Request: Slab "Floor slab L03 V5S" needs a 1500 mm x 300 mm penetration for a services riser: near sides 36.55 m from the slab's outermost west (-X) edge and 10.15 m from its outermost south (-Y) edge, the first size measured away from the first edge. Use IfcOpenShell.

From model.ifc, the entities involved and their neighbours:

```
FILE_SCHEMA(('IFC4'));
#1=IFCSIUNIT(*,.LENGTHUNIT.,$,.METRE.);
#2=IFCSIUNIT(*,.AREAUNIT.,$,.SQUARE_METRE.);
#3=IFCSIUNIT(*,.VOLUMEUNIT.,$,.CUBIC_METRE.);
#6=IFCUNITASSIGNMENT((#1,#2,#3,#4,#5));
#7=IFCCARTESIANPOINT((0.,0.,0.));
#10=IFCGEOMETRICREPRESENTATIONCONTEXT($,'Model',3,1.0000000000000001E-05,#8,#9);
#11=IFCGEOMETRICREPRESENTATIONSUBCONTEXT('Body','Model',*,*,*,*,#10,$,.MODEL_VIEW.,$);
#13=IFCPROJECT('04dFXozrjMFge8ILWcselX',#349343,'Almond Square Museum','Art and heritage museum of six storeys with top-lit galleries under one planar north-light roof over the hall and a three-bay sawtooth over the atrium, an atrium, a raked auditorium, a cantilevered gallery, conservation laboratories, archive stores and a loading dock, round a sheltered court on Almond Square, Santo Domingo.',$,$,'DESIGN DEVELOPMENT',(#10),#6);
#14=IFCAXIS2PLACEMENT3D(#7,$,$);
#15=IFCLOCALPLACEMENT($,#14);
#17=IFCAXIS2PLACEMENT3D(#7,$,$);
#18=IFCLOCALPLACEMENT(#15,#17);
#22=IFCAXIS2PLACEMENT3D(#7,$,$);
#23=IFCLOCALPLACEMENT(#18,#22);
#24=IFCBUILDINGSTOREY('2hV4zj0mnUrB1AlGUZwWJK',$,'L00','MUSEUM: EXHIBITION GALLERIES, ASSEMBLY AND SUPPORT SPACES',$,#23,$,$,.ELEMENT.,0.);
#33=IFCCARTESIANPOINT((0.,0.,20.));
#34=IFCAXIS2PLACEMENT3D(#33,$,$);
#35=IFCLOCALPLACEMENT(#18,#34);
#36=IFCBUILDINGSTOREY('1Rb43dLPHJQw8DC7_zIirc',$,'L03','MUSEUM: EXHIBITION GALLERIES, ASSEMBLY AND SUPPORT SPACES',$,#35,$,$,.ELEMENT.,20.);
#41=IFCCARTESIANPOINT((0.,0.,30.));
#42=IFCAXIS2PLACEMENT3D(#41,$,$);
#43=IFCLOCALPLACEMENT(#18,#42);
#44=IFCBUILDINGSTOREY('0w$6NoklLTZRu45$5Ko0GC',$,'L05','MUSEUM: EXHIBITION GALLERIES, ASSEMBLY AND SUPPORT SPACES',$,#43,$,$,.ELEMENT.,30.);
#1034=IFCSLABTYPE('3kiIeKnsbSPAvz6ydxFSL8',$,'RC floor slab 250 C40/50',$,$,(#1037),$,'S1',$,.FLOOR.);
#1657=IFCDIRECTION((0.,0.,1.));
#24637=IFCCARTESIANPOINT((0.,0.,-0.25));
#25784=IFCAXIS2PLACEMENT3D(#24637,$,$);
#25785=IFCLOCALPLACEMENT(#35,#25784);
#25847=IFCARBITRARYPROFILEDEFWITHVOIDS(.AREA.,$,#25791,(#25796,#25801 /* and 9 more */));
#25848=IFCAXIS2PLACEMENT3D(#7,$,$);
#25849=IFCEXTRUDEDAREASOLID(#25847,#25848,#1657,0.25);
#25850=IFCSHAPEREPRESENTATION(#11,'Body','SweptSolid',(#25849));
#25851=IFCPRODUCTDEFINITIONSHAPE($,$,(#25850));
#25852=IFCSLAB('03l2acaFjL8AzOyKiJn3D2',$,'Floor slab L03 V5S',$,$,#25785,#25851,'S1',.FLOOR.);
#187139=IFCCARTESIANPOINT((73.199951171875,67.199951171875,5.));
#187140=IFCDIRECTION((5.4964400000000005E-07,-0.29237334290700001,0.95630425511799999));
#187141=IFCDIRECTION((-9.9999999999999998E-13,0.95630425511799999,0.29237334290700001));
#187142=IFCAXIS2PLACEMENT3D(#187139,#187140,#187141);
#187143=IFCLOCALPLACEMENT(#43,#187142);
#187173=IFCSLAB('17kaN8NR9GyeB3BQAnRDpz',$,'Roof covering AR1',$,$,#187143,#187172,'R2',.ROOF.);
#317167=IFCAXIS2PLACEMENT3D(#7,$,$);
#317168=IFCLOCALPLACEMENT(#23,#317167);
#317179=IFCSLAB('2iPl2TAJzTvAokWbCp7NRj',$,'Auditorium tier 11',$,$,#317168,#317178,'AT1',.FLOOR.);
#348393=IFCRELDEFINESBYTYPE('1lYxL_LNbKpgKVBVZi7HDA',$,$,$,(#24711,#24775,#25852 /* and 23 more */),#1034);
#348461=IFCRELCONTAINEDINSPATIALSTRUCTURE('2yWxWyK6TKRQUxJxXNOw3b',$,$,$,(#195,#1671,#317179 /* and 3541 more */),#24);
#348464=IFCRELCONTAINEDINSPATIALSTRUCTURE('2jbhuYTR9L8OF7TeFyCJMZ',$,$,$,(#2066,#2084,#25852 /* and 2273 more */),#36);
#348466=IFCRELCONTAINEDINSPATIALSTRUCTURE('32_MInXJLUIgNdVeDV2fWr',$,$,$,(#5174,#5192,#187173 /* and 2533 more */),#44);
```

```python
import numpy as np
import ifcopenshell
import ifcopenshell.api.feature
import ifcopenshell.api.geometry
import ifcopenshell.api.root
import ifcopenshell.geom
import ifcopenshell.util.placement
import ifcopenshell.util.representation
import ifcopenshell.util.shape
import ifcopenshell.util.unit

model = ifcopenshell.open("model.ifc")
unit_scale = ifcopenshell.util.unit.calculate_unit_scale(model)
settings = ifcopenshell.geom.settings()


def volume(element):
    """Net volume in cubic metres, openings subtracted."""
    shape = ifcopenshell.geom.create_shape(settings, element)
    return ifcopenshell.util.shape.get_volume(shape.geometry)


slab = model.by_id(25852)
before = volume(slab)

# Extent in the slab's own axes, in metres. The edges named are its -X and -Y sides.
slab_shape = ifcopenshell.geom.create_shape(settings, slab)
vertices = ifcopenshell.util.shape.get_vertices(slab_shape.geometry)
x_min, y_min, bottom = vertices.min(axis=0)
top = vertices[:, 2].max()

opening = ifcopenshell.api.root.create_entity(model, ifc_class="IfcOpeningElement", name="Services riser opening", predefined_type="OPENING")
context = ifcopenshell.util.representation.get_context(model, "Model", "Body", "MODEL_VIEW")
width, depth = 1.5, 0.3
outline = [(0.0, 0.0), (width, 0.0), (width, depth), (0.0, depth), (0.0, 0.0)]
# Overshoot both faces by 50 mm so the cut is clean.
shape = ifcopenshell.api.geometry.add_slab_representation(
    model, context=context, depth=top - bottom + 0.1, polyline=outline
)
ifcopenshell.api.geometry.assign_representation(model, product=opening, representation=shape)

matrix = ifcopenshell.util.placement.get_local_placement(slab.ObjectPlacement)
matrix[:, 3] = matrix @ np.append(np.array([x_min + 36.55, y_min + 10.15, bottom - 0.05]) / unit_scale, 1.0)
ifcopenshell.api.geometry.edit_object_placement(model, product=opening, matrix=matrix, is_si=False)
ifcopenshell.api.feature.add_feature(model, feature=opening, element=slab)

after = volume(slab)

print(f"slab volume {before:.3f} -> {after:.3f} m3")

model.write("model_edited.ifc")
```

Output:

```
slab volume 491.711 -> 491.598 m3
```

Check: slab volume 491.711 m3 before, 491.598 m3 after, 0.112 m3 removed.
